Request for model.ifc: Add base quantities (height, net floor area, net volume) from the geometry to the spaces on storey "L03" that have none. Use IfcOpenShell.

First a look at what the model holds.

```python
import ifcopenshell
import ifcopenshell.util.element
import ifcopenshell.util.unit

model = ifcopenshell.open("model.ifc")
print(model.schema)
for unit_type in ("LENGTHUNIT", "AREAUNIT", "VOLUMEUNIT"):
    print(unit_type, ifcopenshell.util.unit.calculate_unit_scale(model, unit_type))
storey = next(s for s in model.by_type("IfcBuildingStorey") if s.Name == "L03")
spaces = [e for e in ifcopenshell.util.element.get_decomposition(storey) if e.is_a("IfcSpace")]
for e in sorted(spaces, key=lambda e: e.id()):
    print(e.id(), e.is_a(), e.Name, list(ifcopenshell.util.element.get_psets(e, qtos_only=True)), sep=" | ")
```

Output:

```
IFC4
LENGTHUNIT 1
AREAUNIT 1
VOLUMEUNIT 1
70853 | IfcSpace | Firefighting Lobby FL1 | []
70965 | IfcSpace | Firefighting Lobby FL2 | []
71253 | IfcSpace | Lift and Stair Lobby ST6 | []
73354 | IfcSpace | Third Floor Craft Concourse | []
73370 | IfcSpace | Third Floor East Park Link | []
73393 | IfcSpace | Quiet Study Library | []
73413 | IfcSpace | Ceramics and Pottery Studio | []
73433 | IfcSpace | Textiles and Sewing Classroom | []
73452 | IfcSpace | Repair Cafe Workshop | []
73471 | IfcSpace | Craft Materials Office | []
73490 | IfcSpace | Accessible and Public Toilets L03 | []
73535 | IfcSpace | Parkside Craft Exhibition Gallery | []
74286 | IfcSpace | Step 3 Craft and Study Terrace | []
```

```python
import ifcopenshell
import ifcopenshell.api.pset
import ifcopenshell.geom
import ifcopenshell.util.element
import ifcopenshell.util.shape
import ifcopenshell.util.unit

model = ifcopenshell.open("model.ifc")
unit_scale = ifcopenshell.util.unit.calculate_unit_scale(model)
area_scale = ifcopenshell.util.unit.calculate_unit_scale(model, "AREAUNIT")
volume_scale = ifcopenshell.util.unit.calculate_unit_scale(model, "VOLUMEUNIT")
settings = ifcopenshell.geom.settings()

storey = next(s for s in model.by_type("IfcBuildingStorey") if s.Name == "L03")
spaces = [e for e in ifcopenshell.util.element.get_decomposition(storey) if e.is_a("IfcSpace")]

for e in sorted(spaces, key=lambda e: e.id()):
    if ifcopenshell.util.element.get_psets(e, qtos_only=True, should_inherit=False):
        continue
    # Geometry comes back in metres, in the element's own axes.
    shape = ifcopenshell.geom.create_shape(settings, e)
    values = {
        "Height": ifcopenshell.util.shape.get_z(shape.geometry) / unit_scale,
        "NetFloorArea": ifcopenshell.util.shape.get_footprint_area(shape.geometry) / area_scale,
        "NetVolume": ifcopenshell.util.shape.get_volume(shape.geometry) / volume_scale,
    }
    qto = ifcopenshell.api.pset.add_qto(model, product=e, name="Qto_SpaceBaseQuantities")
    ifcopenshell.api.pset.edit_qto(model, qto=qto, properties=values)
    print(e.id(), {k: round(v, 3) for k, v in values.items()})

model.write("model-out.ifc")
```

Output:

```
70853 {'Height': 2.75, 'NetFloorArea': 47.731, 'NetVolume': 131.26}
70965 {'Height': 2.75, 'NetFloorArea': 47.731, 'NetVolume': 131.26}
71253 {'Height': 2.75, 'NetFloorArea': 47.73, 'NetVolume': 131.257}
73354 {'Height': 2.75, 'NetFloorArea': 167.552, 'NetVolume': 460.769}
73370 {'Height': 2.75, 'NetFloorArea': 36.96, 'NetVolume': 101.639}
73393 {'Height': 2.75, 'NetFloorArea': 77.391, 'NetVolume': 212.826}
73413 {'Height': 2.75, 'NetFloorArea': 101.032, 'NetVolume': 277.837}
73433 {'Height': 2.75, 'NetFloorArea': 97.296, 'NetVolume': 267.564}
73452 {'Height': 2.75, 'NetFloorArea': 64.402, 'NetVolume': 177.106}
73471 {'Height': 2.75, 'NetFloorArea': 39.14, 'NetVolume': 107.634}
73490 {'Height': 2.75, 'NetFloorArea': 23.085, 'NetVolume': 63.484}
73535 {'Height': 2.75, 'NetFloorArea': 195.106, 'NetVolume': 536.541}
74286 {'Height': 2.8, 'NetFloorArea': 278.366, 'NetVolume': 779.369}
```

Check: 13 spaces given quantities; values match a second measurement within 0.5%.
